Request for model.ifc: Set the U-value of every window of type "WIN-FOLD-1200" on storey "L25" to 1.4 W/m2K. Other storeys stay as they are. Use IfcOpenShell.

First a look at what the model holds.

```python
import ifcopenshell
import ifcopenshell.util.element

model = ifcopenshell.open("model.ifc")
print(model.schema)
storey = next(s for s in model.by_type("IfcBuildingStorey") if s.Name == "L25")
windows = [e for e in ifcopenshell.util.element.get_decomposition(storey) if e.is_a("IfcWindow")]
seen = {}
for e in windows:
    element_type = ifcopenshell.util.element.get_type(e)
    key = (element_type.Name if element_type != e and element_type else None, ifcopenshell.util.element.get_pset(e, "Pset_WindowCommon", "ThermalTransmittance"))
    seen[key] = seen.get(key, 0) + 1
for (name, value), count in sorted(seen.items(), key=str):
    print(count, "x", name, "|", value)
```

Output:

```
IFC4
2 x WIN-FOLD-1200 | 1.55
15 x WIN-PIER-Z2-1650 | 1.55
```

```python
import ifcopenshell
import ifcopenshell.api.pset
import ifcopenshell.util.element

model = ifcopenshell.open("model.ifc")

storey = next(s for s in model.by_type("IfcBuildingStorey") if s.Name == "L25")
windows = [e for e in ifcopenshell.util.element.get_decomposition(storey) if e.is_a("IfcWindow")]

count = 0
for e in windows:
    element_type = ifcopenshell.util.element.get_type(e)
    if element_type in (None, e) or element_type.Name != "WIN-FOLD-1200":
        continue
    found = ifcopenshell.util.element.get_pset(e, "Pset_WindowCommon", should_inherit=False)
    if found:
        pset = model.by_id(found["id"])
        if len(ifcopenshell.util.element.get_elements_by_pset(pset)) > 1:
            pset = ifcopenshell.api.pset.unshare_pset(model, products=[e], pset=pset)[0]
    else:
        pset = ifcopenshell.api.pset.add_pset(model, product=e, name="Pset_WindowCommon")
    ifcopenshell.api.pset.edit_pset(model, pset=pset, properties={"ThermalTransmittance": 1.4})
    count += 1

print(count, "windows updated")

model.write("model_updated.ifc")
```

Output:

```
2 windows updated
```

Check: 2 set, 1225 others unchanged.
